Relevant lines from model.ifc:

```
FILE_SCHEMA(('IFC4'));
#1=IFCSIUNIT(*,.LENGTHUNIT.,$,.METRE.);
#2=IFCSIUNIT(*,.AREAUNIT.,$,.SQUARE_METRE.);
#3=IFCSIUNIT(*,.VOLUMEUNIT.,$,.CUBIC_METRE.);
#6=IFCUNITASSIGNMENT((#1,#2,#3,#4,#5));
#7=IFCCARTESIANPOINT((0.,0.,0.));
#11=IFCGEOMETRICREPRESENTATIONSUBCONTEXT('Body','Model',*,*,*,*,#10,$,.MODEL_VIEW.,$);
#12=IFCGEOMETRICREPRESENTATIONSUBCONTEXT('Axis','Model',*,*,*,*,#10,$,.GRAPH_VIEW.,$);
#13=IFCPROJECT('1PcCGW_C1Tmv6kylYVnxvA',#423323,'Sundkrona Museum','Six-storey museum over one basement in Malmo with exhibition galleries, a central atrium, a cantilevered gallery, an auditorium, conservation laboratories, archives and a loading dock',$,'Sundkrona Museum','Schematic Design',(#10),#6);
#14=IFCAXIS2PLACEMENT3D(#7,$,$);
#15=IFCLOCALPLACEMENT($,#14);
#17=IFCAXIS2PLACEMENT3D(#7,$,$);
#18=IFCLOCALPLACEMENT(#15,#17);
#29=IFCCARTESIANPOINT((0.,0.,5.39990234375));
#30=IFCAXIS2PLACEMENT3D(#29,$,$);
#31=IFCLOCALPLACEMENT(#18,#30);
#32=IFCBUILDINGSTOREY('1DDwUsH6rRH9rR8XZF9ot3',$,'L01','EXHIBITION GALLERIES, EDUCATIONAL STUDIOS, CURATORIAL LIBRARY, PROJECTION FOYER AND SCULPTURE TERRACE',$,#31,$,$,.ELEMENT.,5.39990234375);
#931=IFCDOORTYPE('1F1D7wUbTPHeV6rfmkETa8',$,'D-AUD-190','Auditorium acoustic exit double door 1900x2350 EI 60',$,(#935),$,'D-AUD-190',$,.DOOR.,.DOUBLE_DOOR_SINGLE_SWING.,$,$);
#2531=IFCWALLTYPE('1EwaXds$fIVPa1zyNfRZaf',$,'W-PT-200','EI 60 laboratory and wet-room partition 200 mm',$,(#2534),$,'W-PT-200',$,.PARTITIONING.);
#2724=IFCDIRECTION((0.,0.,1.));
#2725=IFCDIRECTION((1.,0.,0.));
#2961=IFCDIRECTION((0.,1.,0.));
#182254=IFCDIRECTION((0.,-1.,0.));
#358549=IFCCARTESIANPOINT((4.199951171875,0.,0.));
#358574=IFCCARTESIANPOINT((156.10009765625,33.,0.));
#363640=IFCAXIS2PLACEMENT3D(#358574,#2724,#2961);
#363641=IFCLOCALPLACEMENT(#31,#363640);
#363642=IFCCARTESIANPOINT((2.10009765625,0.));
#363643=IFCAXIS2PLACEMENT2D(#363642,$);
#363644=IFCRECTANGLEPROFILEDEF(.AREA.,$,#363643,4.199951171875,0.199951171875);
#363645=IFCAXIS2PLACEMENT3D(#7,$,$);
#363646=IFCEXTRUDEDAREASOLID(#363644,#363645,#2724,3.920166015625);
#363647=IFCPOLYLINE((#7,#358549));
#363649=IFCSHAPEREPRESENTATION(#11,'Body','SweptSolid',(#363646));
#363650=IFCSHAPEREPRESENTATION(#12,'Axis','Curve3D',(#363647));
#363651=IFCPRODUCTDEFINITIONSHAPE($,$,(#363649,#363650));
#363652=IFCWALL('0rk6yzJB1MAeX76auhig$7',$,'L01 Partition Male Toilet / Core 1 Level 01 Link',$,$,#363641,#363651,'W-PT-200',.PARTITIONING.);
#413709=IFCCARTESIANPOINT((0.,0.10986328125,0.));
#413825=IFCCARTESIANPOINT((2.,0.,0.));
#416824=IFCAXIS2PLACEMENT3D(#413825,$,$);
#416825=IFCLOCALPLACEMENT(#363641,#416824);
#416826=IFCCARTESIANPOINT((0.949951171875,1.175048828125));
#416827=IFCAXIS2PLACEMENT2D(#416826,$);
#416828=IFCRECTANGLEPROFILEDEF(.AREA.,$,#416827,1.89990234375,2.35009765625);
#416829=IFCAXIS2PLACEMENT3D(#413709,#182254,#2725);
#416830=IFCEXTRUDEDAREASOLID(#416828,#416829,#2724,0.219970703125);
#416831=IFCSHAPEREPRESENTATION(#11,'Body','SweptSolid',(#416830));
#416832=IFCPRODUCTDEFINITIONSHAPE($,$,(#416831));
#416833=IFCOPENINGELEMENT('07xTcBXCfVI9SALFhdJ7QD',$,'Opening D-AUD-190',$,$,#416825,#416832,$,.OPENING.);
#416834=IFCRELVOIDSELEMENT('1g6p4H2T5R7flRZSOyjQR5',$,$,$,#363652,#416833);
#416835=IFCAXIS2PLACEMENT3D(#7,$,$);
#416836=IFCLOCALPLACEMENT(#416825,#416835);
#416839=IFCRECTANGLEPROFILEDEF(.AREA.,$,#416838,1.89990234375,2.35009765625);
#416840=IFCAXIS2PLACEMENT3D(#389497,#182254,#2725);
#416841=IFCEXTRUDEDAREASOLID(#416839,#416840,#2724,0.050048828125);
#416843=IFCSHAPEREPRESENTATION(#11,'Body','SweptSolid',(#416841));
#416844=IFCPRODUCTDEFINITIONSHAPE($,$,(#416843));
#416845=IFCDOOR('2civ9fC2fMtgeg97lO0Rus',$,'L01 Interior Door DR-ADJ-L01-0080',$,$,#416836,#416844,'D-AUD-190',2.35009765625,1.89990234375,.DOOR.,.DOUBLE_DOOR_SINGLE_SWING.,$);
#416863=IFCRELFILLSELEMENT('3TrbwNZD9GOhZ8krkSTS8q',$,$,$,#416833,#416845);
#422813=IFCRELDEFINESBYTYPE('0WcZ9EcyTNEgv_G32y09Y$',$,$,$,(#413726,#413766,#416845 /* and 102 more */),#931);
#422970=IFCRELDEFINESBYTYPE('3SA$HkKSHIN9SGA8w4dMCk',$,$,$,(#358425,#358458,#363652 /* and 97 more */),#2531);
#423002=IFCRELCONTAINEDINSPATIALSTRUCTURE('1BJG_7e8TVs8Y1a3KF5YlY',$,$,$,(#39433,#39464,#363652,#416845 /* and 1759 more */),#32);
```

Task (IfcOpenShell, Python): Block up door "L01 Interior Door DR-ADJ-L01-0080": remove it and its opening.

```python
import ifcopenshell
import ifcopenshell.api.feature
import ifcopenshell.api.root
import ifcopenshell.geom
import ifcopenshell.util.shape

model = ifcopenshell.open("model.ifc")
settings = ifcopenshell.geom.settings()


def volume(element):
    """Net volume in cubic metres, openings subtracted."""
    shape = ifcopenshell.geom.create_shape(settings, element)
    return ifcopenshell.util.shape.get_volume(shape.geometry)


door = model.by_guid("2civ9fC2fMtgeg97lO0Rus")
opening = door.FillsVoids[0].RelatingOpeningElement
wall = opening.VoidsElements[0].RelatingBuildingElement
before = volume(wall)

ifcopenshell.api.root.remove_product(model, product=door)
ifcopenshell.api.feature.remove_feature(model, feature=opening)

after = volume(wall)

print(f"wall volume {before:.3f} -> {after:.3f} m3")

model.write("model_v2.ifc")
```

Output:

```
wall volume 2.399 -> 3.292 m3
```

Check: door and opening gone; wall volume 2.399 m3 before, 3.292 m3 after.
